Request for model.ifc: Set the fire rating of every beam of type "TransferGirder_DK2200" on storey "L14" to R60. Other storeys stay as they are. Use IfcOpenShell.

First a look at what the model holds.

```python
import ifcopenshell
import ifcopenshell.util.element

model = ifcopenshell.open("model.ifc")
print(model.schema)
storey = next(s for s in model.by_type("IfcBuildingStorey") if s.Name == "L14")
beams = [e for e in ifcopenshell.util.element.get_decomposition(storey) if e.is_a("IfcBeam")]
seen = {}
for e in beams:
    element_type = ifcopenshell.util.element.get_type(e)
    key = (element_type.Name if element_type != e and element_type else None, ifcopenshell.util.element.get_pset(e, "Pset_BeamCommon", "FireRating"))
    seen[key] = seen.get(key, 0) + 1
for (name, value), count in sorted(seen.items(), key=str):
    print(count, "x", name, "|", value)
```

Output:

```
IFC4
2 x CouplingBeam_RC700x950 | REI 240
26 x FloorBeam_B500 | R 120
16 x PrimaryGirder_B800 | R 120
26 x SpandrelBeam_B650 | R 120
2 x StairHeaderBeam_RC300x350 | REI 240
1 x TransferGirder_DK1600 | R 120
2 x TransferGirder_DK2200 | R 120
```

```python
import ifcopenshell
import ifcopenshell.api.pset
import ifcopenshell.util.element

model = ifcopenshell.open("model.ifc")

storey = next(s for s in model.by_type("IfcBuildingStorey") if s.Name == "L14")
beams = [e for e in ifcopenshell.util.element.get_decomposition(storey) if e.is_a("IfcBeam")]

count = 0
for e in beams:
    element_type = ifcopenshell.util.element.get_type(e)
    if element_type in (None, e) or element_type.Name != "TransferGirder_DK2200":
        continue
    # add_pset returns the element's existing set when there is one.
    pset = ifcopenshell.api.pset.add_pset(model, product=e, name="Pset_BeamCommon")
    ifcopenshell.api.pset.edit_pset(model, pset=pset, properties={"FireRating": "R60"})
    count += 1

print(count, "beams updated")

model.write("model_rev.ifc")
```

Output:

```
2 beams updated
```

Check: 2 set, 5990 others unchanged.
